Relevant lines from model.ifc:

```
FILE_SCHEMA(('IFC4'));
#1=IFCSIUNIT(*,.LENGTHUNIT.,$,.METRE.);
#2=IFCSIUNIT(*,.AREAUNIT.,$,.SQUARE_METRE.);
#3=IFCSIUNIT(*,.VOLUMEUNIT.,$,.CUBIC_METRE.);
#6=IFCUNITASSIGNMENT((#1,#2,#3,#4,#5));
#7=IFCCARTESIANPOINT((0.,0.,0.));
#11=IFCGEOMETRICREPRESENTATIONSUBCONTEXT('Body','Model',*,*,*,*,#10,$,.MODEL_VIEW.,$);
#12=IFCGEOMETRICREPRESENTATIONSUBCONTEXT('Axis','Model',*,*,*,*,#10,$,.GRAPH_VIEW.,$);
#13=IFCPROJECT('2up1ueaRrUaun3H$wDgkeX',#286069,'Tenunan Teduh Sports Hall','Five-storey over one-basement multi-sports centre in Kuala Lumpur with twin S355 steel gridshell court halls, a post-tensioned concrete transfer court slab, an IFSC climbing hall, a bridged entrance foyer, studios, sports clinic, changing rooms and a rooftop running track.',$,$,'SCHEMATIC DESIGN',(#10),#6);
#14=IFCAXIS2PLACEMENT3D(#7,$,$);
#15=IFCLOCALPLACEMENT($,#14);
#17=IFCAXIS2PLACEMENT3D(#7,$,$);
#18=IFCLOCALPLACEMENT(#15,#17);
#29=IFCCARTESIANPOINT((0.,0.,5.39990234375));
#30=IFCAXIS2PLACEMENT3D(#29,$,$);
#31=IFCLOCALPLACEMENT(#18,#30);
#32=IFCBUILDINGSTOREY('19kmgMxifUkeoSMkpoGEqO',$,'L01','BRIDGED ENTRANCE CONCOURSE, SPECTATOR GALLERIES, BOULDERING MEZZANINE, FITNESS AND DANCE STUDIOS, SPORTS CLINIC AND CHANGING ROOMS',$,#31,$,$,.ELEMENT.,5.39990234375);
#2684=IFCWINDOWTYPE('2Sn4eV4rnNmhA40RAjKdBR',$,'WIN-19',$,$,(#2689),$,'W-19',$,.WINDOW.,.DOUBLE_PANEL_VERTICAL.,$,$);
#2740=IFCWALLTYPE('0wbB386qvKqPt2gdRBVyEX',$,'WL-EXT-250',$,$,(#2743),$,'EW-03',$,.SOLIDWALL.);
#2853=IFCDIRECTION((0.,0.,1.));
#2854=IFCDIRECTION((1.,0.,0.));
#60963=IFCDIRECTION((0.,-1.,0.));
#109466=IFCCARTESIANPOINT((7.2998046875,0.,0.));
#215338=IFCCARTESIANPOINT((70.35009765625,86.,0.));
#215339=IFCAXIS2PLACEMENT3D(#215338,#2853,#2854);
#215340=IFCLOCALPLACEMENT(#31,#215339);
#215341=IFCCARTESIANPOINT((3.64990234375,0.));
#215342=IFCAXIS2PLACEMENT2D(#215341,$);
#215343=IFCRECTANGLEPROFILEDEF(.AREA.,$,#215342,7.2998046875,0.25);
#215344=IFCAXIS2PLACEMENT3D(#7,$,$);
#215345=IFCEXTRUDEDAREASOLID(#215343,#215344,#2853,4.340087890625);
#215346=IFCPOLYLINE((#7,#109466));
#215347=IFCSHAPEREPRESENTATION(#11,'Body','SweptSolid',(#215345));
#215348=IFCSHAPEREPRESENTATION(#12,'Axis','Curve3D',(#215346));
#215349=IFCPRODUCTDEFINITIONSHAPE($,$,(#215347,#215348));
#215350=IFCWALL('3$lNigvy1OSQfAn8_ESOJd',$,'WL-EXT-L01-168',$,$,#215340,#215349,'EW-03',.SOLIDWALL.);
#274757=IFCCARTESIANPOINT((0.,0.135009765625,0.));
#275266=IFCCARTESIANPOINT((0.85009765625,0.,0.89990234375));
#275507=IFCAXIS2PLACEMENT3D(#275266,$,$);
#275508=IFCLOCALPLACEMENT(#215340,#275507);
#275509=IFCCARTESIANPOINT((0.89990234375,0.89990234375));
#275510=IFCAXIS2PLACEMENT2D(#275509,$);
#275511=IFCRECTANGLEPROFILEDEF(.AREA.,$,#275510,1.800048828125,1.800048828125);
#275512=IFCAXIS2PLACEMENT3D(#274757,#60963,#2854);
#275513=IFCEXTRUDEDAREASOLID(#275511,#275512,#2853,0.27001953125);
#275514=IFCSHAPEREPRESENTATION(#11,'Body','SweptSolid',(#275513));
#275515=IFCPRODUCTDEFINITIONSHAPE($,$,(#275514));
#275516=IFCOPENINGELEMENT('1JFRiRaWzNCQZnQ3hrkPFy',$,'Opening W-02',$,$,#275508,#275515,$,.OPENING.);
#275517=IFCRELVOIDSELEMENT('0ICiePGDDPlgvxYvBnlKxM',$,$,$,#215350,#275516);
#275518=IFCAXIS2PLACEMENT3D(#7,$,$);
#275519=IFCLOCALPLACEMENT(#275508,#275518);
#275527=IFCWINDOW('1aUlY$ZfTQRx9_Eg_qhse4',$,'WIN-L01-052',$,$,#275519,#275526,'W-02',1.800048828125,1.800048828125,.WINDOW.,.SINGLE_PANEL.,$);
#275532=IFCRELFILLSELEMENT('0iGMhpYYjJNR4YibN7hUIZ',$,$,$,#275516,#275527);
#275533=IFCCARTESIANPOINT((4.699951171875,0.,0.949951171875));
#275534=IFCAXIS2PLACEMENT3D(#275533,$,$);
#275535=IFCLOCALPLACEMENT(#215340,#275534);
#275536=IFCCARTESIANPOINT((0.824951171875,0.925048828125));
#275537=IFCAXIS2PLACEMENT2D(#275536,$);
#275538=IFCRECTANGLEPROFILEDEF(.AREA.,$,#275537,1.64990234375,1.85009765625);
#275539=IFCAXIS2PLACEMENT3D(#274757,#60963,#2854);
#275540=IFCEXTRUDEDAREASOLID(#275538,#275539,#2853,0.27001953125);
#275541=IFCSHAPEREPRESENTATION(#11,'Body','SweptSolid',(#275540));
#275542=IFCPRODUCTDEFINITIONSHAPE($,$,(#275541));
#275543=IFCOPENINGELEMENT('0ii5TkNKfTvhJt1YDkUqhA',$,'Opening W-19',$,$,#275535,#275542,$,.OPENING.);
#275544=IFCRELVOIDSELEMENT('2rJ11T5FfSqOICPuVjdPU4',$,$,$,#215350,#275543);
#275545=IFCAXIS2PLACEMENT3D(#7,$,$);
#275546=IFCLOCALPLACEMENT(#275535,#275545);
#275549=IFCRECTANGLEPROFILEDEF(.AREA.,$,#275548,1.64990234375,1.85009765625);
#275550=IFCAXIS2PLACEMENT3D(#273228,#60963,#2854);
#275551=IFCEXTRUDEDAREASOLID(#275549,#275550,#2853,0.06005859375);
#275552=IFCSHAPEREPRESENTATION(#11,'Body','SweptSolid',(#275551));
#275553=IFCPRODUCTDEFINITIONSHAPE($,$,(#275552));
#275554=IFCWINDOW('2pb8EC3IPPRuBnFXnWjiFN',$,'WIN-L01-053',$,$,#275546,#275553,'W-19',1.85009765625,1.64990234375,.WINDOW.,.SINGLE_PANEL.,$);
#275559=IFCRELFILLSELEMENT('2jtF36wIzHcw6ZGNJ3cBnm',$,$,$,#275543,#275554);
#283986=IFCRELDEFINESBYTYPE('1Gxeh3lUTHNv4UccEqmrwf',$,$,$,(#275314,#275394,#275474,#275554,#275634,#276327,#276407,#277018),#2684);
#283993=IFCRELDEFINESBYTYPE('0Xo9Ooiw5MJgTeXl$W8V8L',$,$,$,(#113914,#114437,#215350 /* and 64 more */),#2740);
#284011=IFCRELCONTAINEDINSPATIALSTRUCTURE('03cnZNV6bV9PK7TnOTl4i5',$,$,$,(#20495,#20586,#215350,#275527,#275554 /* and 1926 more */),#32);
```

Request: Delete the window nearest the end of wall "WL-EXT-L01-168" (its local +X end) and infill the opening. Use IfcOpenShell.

```python
import ifcopenshell
import ifcopenshell.api.feature
import ifcopenshell.api.root
import ifcopenshell.geom
import ifcopenshell.util.shape

model = ifcopenshell.open("model.ifc")
settings = ifcopenshell.geom.settings()


def volume(element):
    """Net volume in cubic metres, openings subtracted."""
    shape = ifcopenshell.geom.create_shape(settings, element)
    return ifcopenshell.util.shape.get_volume(shape.geometry)


window = model.by_id(275554)
opening = window.FillsVoids[0].RelatingOpeningElement
wall = opening.VoidsElements[0].RelatingBuildingElement
before = volume(wall)

ifcopenshell.api.root.remove_product(model, product=window)
ifcopenshell.api.feature.remove_feature(model, feature=opening)

after = volume(wall)

print(f"wall volume {before:.3f} -> {after:.3f} m3")

model.write("model-out.ifc")
```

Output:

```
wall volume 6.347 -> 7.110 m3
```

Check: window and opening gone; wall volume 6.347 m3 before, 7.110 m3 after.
